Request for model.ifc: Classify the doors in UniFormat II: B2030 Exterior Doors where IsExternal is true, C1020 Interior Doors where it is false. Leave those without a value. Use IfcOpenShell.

First a look at what the model holds.

```python
import ifcopenshell
import ifcopenshell.util.element

model = ifcopenshell.open("model.ifc")
print(model.schema)
print("classifications:", [c.Name for c in model.by_type("IfcClassification")])
values = [ifcopenshell.util.element.get_pset(e, "Pset_DoorCommon", "IsExternal") for e in model.by_type("IfcDoor")]
for value in (True, False, None):
    print("IsExternal", value, values.count(value))
```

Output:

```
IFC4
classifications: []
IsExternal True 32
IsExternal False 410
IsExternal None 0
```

```python
import ifcopenshell
import ifcopenshell.api.classification
import ifcopenshell.util.element

model = ifcopenshell.open("model.ifc")

system = ifcopenshell.api.classification.add_classification(model, classification="UniFormat II")

doors = model.by_type("IfcDoor")
external = {e: ifcopenshell.util.element.get_pset(e, "Pset_DoorCommon", "IsExternal") for e in doors}
for flag, code, name in ((True, "B2030", "Exterior Doors"), (False, "C1020", "Interior Doors")):
    products = [e for e in doors if external[e] is flag]
    ifcopenshell.api.classification.add_reference(
        model, products=products, classification=system, identification=code, name=name
    )
    print(code, len(products))

model.write("model_edited.ifc")
```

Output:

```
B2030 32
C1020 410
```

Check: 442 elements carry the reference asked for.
